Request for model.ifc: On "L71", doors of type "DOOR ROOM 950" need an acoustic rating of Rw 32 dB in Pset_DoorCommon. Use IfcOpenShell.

First a look at what the model holds.

```python
import ifcopenshell
import ifcopenshell.util.element

model = ifcopenshell.open("model.ifc")
print(model.schema)
storey = next(s for s in model.by_type("IfcBuildingStorey") if s.Name == "L71")
doors = [e for e in ifcopenshell.util.element.get_decomposition(storey) if e.is_a("IfcDoor")]
seen = {}
for e in doors:
    element_type = ifcopenshell.util.element.get_type(e)
    key = (element_type.Name if element_type != e and element_type else None, ifcopenshell.util.element.get_pset(e, "Pset_DoorCommon", "AcousticRating"))
    seen[key] = seen.get(key, 0) + 1
for (name, value), count in sorted(seen.items(), key=str):
    print(count, "x", name, "|", value)
```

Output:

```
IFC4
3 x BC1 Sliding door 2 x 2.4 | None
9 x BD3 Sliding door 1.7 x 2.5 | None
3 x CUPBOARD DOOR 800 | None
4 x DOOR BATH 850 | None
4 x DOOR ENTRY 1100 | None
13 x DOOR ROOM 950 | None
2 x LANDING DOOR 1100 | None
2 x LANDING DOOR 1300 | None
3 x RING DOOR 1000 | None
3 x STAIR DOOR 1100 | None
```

```python
import ifcopenshell
import ifcopenshell.api.pset
import ifcopenshell.util.element

model = ifcopenshell.open("model.ifc")

storey = next(s for s in model.by_type("IfcBuildingStorey") if s.Name == "L71")
doors = [e for e in ifcopenshell.util.element.get_decomposition(storey) if e.is_a("IfcDoor")]

count = 0
for e in doors:
    element_type = ifcopenshell.util.element.get_type(e)
    if element_type in (None, e) or element_type.Name != "DOOR ROOM 950":
        continue
    found = ifcopenshell.util.element.get_pset(e, "Pset_DoorCommon", should_inherit=False)
    if found:
        pset = model.by_id(found["id"])
        if len(ifcopenshell.util.element.get_elements_by_pset(pset)) > 1:
            pset = ifcopenshell.api.pset.unshare_pset(model, products=[e], pset=pset)[0]
    else:
        pset = ifcopenshell.api.pset.add_pset(model, product=e, name="Pset_DoorCommon")
    ifcopenshell.api.pset.edit_pset(model, pset=pset, properties={"AcousticRating": "Rw 32 dB"})
    count += 1

print(count, "doors updated")

model.write("model-out.ifc")
```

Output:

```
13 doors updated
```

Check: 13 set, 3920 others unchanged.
